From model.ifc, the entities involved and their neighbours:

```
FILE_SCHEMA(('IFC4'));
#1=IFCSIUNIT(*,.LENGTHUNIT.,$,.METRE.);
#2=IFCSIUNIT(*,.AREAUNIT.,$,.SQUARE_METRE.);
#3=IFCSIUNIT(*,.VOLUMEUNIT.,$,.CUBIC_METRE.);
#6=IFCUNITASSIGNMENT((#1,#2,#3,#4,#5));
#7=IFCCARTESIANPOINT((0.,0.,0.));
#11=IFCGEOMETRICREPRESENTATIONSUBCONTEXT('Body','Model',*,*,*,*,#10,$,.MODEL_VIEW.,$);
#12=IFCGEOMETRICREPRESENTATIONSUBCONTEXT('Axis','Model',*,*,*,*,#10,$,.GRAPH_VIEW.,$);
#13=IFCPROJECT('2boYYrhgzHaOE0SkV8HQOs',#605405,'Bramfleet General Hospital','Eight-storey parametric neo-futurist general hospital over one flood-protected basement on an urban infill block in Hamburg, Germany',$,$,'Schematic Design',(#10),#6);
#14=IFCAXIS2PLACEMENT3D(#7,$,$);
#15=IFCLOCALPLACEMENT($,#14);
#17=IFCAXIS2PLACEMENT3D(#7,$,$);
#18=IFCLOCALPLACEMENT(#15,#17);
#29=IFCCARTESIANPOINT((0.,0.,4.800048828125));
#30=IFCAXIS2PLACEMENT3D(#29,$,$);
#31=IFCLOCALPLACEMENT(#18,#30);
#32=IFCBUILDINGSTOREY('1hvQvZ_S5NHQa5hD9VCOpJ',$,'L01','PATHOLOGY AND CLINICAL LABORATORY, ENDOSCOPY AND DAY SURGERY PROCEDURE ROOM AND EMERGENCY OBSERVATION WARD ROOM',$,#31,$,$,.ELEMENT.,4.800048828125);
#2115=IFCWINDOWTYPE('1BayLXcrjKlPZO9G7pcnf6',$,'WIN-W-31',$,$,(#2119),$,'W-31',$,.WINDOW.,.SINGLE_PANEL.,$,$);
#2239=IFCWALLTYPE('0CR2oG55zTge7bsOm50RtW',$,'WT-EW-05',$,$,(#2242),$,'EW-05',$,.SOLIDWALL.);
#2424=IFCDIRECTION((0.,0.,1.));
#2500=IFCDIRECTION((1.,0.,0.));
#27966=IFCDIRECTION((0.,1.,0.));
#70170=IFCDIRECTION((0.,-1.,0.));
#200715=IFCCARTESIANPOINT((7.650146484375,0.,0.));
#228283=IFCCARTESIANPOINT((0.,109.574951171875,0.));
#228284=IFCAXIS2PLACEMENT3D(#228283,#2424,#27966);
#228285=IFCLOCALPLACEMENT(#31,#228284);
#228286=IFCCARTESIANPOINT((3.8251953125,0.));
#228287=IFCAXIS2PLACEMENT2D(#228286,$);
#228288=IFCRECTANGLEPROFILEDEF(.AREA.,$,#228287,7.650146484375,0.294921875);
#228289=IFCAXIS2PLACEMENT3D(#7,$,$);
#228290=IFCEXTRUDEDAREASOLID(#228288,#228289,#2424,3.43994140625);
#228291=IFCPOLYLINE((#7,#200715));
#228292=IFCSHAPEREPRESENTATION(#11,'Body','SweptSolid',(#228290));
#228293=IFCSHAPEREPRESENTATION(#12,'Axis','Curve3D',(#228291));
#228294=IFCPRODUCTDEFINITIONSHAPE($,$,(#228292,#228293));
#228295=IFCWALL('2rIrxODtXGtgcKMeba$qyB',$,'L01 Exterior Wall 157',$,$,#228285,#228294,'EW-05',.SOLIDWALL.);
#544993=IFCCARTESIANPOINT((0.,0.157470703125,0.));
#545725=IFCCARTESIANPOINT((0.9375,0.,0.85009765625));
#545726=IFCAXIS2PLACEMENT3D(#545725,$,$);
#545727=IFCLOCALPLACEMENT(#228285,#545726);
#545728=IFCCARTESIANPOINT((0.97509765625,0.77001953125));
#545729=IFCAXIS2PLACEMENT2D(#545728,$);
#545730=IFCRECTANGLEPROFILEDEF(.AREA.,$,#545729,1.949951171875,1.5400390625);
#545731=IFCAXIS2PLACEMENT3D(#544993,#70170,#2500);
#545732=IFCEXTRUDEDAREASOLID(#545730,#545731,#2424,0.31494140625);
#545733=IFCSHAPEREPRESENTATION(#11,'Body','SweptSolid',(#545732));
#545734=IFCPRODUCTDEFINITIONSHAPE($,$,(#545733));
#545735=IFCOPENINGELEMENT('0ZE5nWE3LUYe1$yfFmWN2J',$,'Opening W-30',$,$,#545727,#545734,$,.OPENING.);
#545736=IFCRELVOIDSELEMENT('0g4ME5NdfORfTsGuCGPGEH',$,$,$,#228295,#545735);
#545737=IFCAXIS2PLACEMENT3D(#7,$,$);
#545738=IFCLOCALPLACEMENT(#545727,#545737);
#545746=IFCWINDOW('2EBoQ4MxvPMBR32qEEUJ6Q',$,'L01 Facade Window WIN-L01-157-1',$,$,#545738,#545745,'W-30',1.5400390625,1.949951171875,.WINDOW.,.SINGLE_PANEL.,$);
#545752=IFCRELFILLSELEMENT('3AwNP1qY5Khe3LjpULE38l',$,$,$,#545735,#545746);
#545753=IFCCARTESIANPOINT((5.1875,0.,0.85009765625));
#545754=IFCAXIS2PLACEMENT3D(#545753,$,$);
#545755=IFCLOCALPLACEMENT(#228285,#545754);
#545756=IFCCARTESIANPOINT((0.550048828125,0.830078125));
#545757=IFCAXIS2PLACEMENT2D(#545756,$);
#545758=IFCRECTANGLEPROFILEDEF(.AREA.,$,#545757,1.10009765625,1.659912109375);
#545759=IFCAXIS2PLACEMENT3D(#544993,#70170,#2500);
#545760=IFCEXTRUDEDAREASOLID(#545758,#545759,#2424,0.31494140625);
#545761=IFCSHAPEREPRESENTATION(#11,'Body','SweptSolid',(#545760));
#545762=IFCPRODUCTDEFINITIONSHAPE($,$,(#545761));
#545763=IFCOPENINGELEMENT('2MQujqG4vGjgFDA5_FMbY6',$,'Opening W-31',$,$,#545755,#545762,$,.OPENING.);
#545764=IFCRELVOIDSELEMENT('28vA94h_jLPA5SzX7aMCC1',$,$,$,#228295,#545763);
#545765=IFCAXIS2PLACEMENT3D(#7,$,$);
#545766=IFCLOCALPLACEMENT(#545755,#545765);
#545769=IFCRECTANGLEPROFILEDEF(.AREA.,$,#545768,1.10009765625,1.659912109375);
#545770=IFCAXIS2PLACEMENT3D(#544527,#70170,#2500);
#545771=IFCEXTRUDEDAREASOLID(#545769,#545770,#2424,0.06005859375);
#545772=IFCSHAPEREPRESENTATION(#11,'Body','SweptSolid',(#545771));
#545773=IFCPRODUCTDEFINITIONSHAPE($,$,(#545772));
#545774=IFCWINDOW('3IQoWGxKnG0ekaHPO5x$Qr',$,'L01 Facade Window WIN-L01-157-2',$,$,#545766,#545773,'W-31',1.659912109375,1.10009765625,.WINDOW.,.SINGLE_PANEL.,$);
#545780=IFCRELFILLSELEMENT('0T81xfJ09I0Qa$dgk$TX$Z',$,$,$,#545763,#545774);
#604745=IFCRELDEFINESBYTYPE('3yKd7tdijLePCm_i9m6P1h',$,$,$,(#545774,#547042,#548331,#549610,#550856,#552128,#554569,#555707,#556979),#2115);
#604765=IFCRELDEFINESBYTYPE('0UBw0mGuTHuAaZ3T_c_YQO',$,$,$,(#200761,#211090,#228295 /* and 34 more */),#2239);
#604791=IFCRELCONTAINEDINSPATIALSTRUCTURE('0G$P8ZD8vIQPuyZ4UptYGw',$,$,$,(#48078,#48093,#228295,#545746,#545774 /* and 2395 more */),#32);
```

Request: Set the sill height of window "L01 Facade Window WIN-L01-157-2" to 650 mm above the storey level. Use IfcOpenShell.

```python
import numpy as np
import ifcopenshell
import ifcopenshell.api.geometry
import ifcopenshell.geom
import ifcopenshell.util.element
import ifcopenshell.util.placement
import ifcopenshell.util.shape
import ifcopenshell.util.unit

model = ifcopenshell.open("model.ifc")
unit_scale = ifcopenshell.util.unit.calculate_unit_scale(model)

window = model.by_guid("3IQoWGxKnG0ekaHPO5x$Qr")
opening = window.FillsVoids[0].RelatingOpeningElement
storey = ifcopenshell.util.element.get_container(window, ifc_class="IfcBuildingStorey")
level = ifcopenshell.util.placement.get_local_placement(storey.ObjectPlacement)[2, 3]

# The opening's origin need not be at the sill, so measure its lowest point.
shape = ifcopenshell.geom.create_shape(ifcopenshell.geom.settings(), opening)
bottom = ifcopenshell.util.shape.get_shape_bottom_elevation(shape, shape.geometry) / unit_scale
dz = level + 0.65 / unit_scale - bottom

shift = np.array([0.0, 0.0, dz])
# The window is placed relative to its opening, so it follows when the opening moves.
matrix = ifcopenshell.util.placement.get_local_placement(opening.ObjectPlacement)
matrix[:3, 3] += shift
ifcopenshell.api.geometry.edit_object_placement(
    model, product=opening, matrix=matrix, is_si=False, should_transform_children=True
)

print(f"moved by {dz * unit_scale:+.3f} m")

model.write("model_rev.ifc")
```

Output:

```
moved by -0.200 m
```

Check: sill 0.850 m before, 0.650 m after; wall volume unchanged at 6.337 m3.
